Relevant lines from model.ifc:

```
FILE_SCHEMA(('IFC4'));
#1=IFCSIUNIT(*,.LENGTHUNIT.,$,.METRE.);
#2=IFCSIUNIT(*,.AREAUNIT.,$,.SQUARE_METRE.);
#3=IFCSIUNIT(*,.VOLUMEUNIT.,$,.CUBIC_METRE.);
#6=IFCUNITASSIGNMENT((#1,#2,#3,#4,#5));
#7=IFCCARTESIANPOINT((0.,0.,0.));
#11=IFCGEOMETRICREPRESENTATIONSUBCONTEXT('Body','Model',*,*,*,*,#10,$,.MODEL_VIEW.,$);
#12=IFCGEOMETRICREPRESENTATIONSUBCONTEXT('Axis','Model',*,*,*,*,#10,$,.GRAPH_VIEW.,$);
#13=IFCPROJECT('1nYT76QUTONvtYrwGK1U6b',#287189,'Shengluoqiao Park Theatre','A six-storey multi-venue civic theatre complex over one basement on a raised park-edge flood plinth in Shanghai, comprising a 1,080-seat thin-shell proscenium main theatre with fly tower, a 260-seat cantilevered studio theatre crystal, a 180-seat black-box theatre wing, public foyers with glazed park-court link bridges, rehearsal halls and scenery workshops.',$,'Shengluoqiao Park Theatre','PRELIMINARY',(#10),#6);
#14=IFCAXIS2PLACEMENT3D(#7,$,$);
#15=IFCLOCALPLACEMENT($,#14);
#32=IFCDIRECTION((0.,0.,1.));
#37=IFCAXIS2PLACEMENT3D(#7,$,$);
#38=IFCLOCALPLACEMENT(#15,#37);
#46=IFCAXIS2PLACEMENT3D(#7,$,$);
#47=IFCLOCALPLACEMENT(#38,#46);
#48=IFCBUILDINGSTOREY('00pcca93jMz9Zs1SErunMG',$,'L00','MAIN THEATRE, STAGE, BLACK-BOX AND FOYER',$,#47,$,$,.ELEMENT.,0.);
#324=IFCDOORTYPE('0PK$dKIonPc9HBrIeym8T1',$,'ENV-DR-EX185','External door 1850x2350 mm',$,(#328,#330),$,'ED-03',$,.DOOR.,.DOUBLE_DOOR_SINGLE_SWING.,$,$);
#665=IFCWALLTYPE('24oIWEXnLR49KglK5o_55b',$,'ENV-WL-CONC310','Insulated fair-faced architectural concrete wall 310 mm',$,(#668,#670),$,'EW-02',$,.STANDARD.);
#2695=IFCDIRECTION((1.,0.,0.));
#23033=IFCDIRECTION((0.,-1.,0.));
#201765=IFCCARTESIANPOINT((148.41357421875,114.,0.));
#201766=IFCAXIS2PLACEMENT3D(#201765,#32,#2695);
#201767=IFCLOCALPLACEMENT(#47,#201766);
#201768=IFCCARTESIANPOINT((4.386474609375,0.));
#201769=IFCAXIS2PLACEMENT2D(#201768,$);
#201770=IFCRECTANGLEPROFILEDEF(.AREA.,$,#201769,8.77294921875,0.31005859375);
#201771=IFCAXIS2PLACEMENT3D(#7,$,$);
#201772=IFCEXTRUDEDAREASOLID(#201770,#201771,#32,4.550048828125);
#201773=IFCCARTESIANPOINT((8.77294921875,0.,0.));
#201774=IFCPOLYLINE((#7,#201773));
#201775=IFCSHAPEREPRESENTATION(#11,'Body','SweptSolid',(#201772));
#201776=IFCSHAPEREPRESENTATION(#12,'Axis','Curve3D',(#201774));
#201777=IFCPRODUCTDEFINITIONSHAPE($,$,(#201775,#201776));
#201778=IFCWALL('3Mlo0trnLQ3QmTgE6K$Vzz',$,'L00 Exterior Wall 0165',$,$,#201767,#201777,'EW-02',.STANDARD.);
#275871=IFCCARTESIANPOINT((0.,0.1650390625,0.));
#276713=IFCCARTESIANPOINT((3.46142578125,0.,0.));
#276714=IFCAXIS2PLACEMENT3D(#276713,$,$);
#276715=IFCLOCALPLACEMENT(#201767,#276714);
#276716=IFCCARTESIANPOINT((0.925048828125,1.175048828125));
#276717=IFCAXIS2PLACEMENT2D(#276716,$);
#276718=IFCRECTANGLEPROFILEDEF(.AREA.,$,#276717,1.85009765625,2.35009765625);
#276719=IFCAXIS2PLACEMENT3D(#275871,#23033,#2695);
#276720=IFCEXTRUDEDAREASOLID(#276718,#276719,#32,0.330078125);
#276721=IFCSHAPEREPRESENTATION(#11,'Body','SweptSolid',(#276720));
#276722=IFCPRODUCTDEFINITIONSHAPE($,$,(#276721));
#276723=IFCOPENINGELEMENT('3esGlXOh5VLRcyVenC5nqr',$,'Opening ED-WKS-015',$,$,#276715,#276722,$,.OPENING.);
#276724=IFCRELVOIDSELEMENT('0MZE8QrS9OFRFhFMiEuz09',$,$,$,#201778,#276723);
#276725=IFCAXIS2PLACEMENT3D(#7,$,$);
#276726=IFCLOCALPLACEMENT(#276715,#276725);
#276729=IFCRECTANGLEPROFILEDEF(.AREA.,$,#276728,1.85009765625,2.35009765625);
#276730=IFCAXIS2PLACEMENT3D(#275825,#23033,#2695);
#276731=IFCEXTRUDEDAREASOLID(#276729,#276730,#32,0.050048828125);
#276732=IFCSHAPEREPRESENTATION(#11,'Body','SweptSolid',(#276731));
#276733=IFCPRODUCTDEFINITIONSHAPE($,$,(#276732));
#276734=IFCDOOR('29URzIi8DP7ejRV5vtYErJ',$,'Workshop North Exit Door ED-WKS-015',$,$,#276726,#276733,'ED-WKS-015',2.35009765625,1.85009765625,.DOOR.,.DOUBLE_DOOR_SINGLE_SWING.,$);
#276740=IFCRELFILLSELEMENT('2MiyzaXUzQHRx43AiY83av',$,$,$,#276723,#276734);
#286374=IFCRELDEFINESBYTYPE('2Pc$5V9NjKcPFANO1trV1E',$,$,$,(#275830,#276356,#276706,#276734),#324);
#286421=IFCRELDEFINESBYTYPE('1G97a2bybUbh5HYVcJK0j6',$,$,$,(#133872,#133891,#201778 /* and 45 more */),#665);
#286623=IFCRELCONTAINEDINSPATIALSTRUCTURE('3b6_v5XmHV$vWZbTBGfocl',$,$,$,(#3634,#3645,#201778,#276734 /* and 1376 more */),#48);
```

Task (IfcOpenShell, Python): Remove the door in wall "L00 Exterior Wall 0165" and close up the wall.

```python
import ifcopenshell
import ifcopenshell.api.feature
import ifcopenshell.api.root
import ifcopenshell.geom
import ifcopenshell.util.shape

model = ifcopenshell.open("model.ifc")
settings = ifcopenshell.geom.settings()


def volume(element):
    """Net volume in cubic metres, openings subtracted."""
    shape = ifcopenshell.geom.create_shape(settings, element)
    return ifcopenshell.util.shape.get_volume(shape.geometry)


door = model.by_id(276734)
opening = door.FillsVoids[0].RelatingOpeningElement
wall = opening.VoidsElements[0].RelatingBuildingElement
before = volume(wall)

ifcopenshell.api.root.remove_product(model, product=door)
ifcopenshell.api.feature.remove_feature(model, feature=opening)

after = volume(wall)

print(f"wall volume {before:.3f} -> {after:.3f} m3")

model.write("model_edited.ifc")
```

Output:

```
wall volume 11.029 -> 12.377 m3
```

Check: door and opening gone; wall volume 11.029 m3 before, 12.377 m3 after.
